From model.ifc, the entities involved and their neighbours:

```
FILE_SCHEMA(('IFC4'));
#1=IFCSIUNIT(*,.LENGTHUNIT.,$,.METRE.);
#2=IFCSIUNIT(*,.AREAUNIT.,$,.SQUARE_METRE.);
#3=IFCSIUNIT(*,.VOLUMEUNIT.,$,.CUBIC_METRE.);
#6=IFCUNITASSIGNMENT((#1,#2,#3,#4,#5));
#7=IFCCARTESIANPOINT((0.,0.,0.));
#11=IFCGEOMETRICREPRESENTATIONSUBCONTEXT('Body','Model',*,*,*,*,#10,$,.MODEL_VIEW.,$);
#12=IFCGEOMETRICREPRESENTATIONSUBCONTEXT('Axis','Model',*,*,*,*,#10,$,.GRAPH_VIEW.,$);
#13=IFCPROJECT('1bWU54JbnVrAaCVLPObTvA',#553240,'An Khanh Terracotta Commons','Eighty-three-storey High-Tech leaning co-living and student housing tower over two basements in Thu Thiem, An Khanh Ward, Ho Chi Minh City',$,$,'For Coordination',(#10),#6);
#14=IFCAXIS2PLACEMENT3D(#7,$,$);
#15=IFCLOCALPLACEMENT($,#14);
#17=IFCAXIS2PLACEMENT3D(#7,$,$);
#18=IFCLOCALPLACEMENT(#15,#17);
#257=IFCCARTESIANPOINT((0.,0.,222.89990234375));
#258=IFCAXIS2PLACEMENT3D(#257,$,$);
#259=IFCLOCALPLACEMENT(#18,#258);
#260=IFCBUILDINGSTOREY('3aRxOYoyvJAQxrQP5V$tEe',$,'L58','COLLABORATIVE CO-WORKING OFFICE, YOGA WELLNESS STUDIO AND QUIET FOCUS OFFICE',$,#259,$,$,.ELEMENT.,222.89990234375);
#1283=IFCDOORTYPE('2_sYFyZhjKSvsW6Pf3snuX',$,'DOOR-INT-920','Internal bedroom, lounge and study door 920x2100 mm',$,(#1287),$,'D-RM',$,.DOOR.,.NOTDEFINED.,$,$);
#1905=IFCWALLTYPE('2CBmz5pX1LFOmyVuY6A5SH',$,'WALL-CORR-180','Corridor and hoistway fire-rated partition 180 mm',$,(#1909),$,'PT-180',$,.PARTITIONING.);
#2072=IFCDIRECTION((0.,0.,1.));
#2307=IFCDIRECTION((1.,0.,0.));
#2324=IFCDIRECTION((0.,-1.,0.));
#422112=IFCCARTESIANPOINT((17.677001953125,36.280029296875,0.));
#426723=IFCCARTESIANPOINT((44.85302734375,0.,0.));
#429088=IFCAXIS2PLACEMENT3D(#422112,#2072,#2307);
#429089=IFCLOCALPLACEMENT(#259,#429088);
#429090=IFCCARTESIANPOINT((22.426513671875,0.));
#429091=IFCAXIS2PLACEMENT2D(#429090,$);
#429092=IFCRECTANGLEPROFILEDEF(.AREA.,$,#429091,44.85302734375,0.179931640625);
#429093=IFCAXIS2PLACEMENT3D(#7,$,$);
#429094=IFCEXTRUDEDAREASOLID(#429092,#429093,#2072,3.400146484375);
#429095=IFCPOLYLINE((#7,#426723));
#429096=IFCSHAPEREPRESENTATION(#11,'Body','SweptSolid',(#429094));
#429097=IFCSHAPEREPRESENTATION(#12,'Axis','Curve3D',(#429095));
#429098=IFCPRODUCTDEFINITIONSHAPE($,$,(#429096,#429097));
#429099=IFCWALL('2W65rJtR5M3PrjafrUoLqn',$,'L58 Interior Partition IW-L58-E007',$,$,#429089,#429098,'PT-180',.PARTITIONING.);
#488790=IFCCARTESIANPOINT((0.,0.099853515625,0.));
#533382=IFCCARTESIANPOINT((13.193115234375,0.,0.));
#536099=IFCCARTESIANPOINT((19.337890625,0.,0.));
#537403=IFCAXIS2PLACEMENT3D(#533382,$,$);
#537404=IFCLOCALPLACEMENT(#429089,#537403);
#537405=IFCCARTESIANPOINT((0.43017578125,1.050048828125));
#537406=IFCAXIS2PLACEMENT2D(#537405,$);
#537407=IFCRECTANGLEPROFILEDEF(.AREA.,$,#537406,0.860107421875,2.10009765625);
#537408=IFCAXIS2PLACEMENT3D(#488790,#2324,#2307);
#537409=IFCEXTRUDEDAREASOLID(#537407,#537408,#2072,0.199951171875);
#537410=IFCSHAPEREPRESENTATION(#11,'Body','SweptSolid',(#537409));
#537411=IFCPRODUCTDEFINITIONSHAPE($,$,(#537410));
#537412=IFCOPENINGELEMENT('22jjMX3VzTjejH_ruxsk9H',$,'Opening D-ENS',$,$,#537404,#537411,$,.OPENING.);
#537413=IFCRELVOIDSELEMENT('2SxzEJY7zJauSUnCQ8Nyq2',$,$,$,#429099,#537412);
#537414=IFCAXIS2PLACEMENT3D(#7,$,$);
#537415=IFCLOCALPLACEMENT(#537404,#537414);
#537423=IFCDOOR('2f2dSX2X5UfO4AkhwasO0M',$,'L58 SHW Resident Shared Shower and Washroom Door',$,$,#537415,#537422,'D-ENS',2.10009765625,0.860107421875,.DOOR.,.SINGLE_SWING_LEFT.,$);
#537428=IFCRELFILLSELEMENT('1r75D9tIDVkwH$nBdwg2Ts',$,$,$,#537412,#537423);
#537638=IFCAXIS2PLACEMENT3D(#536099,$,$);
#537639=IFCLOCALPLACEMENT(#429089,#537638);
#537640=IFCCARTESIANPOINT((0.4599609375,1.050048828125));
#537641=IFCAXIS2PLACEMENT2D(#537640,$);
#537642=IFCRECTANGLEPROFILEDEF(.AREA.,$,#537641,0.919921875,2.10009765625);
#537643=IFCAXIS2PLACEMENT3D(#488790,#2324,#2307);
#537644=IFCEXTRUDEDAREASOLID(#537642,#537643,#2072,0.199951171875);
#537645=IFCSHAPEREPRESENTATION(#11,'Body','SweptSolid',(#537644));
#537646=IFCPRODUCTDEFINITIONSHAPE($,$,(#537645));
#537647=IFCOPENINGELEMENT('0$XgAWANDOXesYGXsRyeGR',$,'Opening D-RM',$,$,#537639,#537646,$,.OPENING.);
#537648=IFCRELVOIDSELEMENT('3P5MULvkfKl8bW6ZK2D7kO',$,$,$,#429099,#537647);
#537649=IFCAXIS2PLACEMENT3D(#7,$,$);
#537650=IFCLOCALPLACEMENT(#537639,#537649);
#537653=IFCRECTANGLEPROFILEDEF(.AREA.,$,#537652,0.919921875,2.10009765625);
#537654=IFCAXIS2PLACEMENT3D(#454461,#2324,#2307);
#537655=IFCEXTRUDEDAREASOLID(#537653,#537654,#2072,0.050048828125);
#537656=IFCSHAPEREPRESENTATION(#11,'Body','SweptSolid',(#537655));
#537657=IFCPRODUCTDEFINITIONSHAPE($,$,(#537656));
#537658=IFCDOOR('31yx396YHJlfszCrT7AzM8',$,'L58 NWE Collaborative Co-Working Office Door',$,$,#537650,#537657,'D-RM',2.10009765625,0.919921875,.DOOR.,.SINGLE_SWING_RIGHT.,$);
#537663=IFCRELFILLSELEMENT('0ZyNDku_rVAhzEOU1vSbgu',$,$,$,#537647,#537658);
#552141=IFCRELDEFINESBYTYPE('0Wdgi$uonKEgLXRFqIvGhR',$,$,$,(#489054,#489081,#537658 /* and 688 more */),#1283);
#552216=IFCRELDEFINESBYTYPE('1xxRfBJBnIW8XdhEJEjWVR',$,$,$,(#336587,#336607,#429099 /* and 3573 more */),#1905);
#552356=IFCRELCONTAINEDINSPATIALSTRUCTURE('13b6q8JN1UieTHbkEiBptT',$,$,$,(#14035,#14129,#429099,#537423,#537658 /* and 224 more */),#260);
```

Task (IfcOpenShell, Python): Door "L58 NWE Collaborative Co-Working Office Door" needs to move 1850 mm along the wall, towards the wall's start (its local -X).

```python
import ifcopenshell
import ifcopenshell.api.geometry
import ifcopenshell.util.placement

model = ifcopenshell.open("model.ifc")

door = model.by_guid("31yx396YHJlfszCrT7AzM8")
opening = door.FillsVoids[0].RelatingOpeningElement
wall = opening.VoidsElements[0].RelatingBuildingElement

wall_matrix = ifcopenshell.util.placement.get_local_placement(wall.ObjectPlacement)
shift = wall_matrix[:3, 0] * -1.85
before = ifcopenshell.util.placement.get_local_placement(door.ObjectPlacement)[:3, 3].copy()

# The door is placed relative to its opening, so it follows when the opening moves.
matrix = ifcopenshell.util.placement.get_local_placement(opening.ObjectPlacement)
matrix[:3, 3] += shift
ifcopenshell.api.geometry.edit_object_placement(
    model, product=opening, matrix=matrix, is_si=False, should_transform_children=True
)

after = ifcopenshell.util.placement.get_local_placement(door.ObjectPlacement)[:3, 3]
print("door moved by", (after - before).round(3) + 0.0)

model.write("model_updated.ifc")
```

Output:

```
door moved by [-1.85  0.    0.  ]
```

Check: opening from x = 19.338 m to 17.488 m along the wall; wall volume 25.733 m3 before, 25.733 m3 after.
